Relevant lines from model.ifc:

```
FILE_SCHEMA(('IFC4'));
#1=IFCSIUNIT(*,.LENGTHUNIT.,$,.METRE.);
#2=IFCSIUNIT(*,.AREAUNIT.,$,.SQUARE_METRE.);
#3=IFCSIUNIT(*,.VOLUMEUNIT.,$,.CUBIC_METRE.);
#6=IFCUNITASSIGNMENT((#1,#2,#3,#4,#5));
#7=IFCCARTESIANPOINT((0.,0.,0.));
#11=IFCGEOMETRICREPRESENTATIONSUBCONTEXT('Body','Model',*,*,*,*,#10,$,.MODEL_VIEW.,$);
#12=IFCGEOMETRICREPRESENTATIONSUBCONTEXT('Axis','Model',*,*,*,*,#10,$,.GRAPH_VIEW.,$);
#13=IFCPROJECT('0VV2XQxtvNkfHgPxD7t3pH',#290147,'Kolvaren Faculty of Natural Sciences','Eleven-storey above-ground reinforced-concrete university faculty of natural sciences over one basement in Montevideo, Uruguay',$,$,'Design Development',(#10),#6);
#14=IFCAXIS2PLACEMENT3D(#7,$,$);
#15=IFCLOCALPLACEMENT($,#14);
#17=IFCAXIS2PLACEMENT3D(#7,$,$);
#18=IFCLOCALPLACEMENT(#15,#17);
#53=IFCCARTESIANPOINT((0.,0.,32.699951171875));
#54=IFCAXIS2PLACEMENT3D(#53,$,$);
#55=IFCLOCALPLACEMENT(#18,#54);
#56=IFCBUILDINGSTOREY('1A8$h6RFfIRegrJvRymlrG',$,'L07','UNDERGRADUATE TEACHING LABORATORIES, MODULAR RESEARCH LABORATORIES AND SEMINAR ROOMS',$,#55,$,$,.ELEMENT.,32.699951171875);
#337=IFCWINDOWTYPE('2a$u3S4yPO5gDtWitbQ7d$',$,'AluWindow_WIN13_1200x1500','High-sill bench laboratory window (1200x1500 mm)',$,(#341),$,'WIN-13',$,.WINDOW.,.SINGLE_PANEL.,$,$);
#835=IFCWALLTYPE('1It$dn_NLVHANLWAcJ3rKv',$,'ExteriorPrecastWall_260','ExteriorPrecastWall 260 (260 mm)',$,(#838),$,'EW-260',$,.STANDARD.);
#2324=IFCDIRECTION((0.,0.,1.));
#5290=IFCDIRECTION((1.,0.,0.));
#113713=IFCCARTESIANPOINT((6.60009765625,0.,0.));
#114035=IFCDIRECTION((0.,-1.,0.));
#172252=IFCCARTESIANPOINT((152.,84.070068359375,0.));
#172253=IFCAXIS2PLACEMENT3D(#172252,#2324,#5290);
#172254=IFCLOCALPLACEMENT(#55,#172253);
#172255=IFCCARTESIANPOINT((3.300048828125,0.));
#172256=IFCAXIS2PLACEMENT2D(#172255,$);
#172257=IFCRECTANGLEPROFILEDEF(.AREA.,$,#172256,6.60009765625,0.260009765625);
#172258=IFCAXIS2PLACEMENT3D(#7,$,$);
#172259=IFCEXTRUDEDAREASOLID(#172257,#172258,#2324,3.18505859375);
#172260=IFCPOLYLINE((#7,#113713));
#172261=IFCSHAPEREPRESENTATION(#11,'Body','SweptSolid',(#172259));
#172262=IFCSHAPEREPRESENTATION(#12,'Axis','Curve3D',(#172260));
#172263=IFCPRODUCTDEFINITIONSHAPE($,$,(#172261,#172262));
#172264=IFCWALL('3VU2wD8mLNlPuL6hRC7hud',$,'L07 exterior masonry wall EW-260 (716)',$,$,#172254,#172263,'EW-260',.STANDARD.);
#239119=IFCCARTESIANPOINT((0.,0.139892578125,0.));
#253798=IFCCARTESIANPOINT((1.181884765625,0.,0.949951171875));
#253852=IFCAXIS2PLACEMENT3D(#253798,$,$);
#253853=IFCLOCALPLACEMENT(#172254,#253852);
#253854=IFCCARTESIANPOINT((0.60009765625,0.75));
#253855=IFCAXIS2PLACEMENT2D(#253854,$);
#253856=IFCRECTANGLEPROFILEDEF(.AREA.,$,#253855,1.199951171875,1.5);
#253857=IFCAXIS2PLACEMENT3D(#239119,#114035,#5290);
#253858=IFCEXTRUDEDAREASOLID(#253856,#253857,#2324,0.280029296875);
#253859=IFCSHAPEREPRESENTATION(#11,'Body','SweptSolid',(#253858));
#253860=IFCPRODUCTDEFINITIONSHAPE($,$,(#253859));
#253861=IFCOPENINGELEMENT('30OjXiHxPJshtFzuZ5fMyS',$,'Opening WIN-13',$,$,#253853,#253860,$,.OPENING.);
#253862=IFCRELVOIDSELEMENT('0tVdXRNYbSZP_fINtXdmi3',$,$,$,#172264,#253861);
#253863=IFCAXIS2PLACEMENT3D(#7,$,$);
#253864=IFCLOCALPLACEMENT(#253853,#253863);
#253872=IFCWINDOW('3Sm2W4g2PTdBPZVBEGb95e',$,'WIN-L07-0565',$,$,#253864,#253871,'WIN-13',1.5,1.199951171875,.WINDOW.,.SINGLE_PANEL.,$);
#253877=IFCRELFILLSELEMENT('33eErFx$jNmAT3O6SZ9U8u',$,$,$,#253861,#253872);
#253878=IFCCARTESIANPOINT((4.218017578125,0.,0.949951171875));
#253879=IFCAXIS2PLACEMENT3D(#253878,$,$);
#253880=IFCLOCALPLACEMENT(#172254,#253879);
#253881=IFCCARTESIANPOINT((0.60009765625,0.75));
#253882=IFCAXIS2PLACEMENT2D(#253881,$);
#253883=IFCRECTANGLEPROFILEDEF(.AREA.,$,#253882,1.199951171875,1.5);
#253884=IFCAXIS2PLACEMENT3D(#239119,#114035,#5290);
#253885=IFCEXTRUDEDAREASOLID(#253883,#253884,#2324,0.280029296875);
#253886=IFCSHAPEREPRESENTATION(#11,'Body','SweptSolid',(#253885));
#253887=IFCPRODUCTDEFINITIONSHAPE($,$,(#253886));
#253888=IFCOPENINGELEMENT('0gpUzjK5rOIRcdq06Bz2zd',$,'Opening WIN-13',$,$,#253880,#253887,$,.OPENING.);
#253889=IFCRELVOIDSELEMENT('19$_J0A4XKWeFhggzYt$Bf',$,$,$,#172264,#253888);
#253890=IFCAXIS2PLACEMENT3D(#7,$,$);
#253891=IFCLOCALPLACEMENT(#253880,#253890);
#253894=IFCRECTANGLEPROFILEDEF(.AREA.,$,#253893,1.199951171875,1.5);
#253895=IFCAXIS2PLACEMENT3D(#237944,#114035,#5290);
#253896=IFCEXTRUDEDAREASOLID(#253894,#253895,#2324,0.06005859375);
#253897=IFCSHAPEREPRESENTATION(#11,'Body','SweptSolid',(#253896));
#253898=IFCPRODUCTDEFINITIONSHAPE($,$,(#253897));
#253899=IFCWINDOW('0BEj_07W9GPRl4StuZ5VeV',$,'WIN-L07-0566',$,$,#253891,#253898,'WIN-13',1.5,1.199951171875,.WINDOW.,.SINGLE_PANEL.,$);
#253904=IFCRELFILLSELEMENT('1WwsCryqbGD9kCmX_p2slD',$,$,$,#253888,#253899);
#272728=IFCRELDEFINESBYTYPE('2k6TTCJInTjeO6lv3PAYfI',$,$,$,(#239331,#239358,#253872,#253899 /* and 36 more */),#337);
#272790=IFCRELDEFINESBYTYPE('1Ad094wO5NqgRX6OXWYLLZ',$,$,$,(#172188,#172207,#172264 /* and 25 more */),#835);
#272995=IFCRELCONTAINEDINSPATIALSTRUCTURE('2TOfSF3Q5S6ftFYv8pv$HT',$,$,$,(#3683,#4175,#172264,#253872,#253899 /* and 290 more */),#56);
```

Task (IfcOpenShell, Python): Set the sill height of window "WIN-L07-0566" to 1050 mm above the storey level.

```python
import numpy as np
import ifcopenshell
import ifcopenshell.api.geometry
import ifcopenshell.geom
import ifcopenshell.util.element
import ifcopenshell.util.placement
import ifcopenshell.util.shape
import ifcopenshell.util.unit

model = ifcopenshell.open("model.ifc")
unit_scale = ifcopenshell.util.unit.calculate_unit_scale(model)

window = model.by_guid("0BEj_07W9GPRl4StuZ5VeV")
opening = window.FillsVoids[0].RelatingOpeningElement
storey = ifcopenshell.util.element.get_container(window, ifc_class="IfcBuildingStorey")
level = ifcopenshell.util.placement.get_local_placement(storey.ObjectPlacement)[2, 3]

# The opening's origin need not be at the sill, so measure its lowest point.
shape = ifcopenshell.geom.create_shape(ifcopenshell.geom.settings(), opening)
bottom = ifcopenshell.util.shape.get_shape_bottom_elevation(shape, shape.geometry) / unit_scale
dz = level + 1.05 / unit_scale - bottom

shift = np.array([0.0, 0.0, dz])
# The window is placed relative to its opening, so it follows when the opening moves.
matrix = ifcopenshell.util.placement.get_local_placement(opening.ObjectPlacement)
matrix[:3, 3] += shift
ifcopenshell.api.geometry.edit_object_placement(
    model, product=opening, matrix=matrix, is_si=False, should_transform_children=True
)

print(f"moved by {dz * unit_scale:+.3f} m")

model.write("model-out.ifc")
```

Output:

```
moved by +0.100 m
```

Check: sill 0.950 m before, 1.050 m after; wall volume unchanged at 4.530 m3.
